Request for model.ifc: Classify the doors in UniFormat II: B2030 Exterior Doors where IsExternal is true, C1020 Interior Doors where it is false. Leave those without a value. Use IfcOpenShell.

First a look at what the model holds.

```python
import ifcopenshell
import ifcopenshell.util.element

model = ifcopenshell.open("model.ifc")
print(model.schema)
print("classifications:", [c.Name for c in model.by_type("IfcClassification")])
values = [ifcopenshell.util.element.get_pset(e, "Pset_DoorCommon", "IsExternal") for e in model.by_type("IfcDoor")]
for value in (True, False, None):
    print("IsExternal", value, values.count(value))
```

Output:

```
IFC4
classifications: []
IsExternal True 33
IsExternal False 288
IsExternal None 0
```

```python
import ifcopenshell
import ifcopenshell.api.classification
import ifcopenshell.util.element

model = ifcopenshell.open("model.ifc")

system = ifcopenshell.api.classification.add_classification(model, classification="UniFormat II")

doors = model.by_type("IfcDoor")
external = {e: ifcopenshell.util.element.get_pset(e, "Pset_DoorCommon", "IsExternal") for e in doors}
for flag, code, name in ((True, "B2030", "Exterior Doors"), (False, "C1020", "Interior Doors")):
    products = [e for e in doors if external[e] is flag]
    ifcopenshell.api.classification.add_reference(
        model, products=products, classification=system, identification=code, name=name
    )
    print(code, len(products))

model.write("model_updated.ifc")
```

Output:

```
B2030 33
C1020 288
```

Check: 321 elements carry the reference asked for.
